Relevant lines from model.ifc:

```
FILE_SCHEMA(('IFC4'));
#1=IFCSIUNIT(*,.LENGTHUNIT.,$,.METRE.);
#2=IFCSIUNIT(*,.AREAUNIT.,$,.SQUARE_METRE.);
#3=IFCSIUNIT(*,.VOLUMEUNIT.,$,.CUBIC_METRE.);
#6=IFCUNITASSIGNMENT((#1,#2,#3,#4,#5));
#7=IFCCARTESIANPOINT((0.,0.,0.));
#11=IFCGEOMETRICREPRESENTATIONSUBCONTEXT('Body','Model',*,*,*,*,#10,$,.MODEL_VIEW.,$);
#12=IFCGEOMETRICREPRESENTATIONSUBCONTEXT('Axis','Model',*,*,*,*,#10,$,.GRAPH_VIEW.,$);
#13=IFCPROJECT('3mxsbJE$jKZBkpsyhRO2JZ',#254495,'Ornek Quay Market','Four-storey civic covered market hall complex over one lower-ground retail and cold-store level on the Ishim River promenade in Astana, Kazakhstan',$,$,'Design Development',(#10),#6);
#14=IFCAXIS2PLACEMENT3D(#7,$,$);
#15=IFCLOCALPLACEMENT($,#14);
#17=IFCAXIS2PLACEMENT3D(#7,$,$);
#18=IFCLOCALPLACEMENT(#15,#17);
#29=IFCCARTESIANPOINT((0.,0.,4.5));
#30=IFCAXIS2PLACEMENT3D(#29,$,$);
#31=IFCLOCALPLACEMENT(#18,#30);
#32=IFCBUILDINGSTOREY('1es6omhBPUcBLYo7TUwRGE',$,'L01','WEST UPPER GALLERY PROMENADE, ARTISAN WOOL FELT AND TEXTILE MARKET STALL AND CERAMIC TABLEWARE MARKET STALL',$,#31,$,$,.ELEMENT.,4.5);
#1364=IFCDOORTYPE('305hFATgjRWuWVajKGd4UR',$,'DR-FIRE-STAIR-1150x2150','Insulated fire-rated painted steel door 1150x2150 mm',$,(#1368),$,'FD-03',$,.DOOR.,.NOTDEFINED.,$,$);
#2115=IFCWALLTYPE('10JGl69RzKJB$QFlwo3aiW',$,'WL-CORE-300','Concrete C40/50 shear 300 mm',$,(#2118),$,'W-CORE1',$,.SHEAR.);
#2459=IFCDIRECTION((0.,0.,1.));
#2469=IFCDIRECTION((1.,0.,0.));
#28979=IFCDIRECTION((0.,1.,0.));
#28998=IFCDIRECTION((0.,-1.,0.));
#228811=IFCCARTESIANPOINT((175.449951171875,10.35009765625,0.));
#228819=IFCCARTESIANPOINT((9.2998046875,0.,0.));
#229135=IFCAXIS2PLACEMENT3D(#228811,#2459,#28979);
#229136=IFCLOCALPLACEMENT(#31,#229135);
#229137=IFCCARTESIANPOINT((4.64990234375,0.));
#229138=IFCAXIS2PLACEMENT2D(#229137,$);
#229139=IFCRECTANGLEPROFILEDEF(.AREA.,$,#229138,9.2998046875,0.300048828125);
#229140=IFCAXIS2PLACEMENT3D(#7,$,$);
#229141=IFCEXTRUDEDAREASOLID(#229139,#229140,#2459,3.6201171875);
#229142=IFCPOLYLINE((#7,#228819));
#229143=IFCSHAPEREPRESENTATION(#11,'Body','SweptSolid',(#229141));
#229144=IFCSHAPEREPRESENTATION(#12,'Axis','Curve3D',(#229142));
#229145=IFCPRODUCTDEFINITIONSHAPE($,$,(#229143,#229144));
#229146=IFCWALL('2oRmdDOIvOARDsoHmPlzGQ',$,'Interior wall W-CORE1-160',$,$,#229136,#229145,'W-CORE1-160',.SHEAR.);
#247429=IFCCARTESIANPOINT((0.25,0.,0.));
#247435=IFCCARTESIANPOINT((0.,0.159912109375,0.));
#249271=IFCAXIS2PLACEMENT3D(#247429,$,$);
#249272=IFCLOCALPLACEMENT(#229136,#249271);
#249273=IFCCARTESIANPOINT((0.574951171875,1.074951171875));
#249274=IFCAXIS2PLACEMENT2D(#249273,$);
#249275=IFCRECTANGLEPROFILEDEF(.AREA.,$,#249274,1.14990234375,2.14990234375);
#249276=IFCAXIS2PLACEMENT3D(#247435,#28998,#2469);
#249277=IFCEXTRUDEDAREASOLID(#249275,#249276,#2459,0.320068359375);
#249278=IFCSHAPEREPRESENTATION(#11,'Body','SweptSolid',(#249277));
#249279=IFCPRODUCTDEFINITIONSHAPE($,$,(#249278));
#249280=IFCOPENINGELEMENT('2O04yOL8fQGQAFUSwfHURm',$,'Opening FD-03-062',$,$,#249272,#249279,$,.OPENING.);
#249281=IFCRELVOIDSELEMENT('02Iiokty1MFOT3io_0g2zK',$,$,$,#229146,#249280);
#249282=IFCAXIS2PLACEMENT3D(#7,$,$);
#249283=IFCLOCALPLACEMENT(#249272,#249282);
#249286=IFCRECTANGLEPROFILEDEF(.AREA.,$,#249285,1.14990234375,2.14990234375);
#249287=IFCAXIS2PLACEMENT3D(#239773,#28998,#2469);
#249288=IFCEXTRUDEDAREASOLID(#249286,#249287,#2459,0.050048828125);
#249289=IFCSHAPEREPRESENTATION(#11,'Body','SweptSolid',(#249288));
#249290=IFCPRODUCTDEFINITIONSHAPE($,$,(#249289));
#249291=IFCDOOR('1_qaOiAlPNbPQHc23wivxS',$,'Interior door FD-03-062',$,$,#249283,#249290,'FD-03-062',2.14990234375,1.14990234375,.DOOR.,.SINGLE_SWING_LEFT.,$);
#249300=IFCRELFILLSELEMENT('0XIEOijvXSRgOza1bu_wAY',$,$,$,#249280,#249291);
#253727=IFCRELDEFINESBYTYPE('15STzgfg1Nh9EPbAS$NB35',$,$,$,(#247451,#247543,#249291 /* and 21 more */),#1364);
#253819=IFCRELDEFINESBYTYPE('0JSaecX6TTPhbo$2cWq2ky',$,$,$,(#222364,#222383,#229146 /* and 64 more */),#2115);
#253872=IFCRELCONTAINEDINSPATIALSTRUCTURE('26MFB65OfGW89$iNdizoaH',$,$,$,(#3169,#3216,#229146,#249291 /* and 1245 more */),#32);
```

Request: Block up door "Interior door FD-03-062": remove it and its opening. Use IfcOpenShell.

```python
import ifcopenshell
import ifcopenshell.api.feature
import ifcopenshell.api.root
import ifcopenshell.geom
import ifcopenshell.util.shape

model = ifcopenshell.open("model.ifc")
settings = ifcopenshell.geom.settings()


def volume(element):
    """Net volume in cubic metres, openings subtracted."""
    shape = ifcopenshell.geom.create_shape(settings, element)
    return ifcopenshell.util.shape.get_volume(shape.geometry)


door = model.by_id(249291)
opening = door.FillsVoids[0].RelatingOpeningElement
wall = opening.VoidsElements[0].RelatingBuildingElement
before = volume(wall)

ifcopenshell.api.root.remove_product(model, product=door)
ifcopenshell.api.feature.remove_feature(model, feature=opening)

after = volume(wall)

print(f"wall volume {before:.3f} -> {after:.3f} m3")

model.write("model_rev.ifc")
```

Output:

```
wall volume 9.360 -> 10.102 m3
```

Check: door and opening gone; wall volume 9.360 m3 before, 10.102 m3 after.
